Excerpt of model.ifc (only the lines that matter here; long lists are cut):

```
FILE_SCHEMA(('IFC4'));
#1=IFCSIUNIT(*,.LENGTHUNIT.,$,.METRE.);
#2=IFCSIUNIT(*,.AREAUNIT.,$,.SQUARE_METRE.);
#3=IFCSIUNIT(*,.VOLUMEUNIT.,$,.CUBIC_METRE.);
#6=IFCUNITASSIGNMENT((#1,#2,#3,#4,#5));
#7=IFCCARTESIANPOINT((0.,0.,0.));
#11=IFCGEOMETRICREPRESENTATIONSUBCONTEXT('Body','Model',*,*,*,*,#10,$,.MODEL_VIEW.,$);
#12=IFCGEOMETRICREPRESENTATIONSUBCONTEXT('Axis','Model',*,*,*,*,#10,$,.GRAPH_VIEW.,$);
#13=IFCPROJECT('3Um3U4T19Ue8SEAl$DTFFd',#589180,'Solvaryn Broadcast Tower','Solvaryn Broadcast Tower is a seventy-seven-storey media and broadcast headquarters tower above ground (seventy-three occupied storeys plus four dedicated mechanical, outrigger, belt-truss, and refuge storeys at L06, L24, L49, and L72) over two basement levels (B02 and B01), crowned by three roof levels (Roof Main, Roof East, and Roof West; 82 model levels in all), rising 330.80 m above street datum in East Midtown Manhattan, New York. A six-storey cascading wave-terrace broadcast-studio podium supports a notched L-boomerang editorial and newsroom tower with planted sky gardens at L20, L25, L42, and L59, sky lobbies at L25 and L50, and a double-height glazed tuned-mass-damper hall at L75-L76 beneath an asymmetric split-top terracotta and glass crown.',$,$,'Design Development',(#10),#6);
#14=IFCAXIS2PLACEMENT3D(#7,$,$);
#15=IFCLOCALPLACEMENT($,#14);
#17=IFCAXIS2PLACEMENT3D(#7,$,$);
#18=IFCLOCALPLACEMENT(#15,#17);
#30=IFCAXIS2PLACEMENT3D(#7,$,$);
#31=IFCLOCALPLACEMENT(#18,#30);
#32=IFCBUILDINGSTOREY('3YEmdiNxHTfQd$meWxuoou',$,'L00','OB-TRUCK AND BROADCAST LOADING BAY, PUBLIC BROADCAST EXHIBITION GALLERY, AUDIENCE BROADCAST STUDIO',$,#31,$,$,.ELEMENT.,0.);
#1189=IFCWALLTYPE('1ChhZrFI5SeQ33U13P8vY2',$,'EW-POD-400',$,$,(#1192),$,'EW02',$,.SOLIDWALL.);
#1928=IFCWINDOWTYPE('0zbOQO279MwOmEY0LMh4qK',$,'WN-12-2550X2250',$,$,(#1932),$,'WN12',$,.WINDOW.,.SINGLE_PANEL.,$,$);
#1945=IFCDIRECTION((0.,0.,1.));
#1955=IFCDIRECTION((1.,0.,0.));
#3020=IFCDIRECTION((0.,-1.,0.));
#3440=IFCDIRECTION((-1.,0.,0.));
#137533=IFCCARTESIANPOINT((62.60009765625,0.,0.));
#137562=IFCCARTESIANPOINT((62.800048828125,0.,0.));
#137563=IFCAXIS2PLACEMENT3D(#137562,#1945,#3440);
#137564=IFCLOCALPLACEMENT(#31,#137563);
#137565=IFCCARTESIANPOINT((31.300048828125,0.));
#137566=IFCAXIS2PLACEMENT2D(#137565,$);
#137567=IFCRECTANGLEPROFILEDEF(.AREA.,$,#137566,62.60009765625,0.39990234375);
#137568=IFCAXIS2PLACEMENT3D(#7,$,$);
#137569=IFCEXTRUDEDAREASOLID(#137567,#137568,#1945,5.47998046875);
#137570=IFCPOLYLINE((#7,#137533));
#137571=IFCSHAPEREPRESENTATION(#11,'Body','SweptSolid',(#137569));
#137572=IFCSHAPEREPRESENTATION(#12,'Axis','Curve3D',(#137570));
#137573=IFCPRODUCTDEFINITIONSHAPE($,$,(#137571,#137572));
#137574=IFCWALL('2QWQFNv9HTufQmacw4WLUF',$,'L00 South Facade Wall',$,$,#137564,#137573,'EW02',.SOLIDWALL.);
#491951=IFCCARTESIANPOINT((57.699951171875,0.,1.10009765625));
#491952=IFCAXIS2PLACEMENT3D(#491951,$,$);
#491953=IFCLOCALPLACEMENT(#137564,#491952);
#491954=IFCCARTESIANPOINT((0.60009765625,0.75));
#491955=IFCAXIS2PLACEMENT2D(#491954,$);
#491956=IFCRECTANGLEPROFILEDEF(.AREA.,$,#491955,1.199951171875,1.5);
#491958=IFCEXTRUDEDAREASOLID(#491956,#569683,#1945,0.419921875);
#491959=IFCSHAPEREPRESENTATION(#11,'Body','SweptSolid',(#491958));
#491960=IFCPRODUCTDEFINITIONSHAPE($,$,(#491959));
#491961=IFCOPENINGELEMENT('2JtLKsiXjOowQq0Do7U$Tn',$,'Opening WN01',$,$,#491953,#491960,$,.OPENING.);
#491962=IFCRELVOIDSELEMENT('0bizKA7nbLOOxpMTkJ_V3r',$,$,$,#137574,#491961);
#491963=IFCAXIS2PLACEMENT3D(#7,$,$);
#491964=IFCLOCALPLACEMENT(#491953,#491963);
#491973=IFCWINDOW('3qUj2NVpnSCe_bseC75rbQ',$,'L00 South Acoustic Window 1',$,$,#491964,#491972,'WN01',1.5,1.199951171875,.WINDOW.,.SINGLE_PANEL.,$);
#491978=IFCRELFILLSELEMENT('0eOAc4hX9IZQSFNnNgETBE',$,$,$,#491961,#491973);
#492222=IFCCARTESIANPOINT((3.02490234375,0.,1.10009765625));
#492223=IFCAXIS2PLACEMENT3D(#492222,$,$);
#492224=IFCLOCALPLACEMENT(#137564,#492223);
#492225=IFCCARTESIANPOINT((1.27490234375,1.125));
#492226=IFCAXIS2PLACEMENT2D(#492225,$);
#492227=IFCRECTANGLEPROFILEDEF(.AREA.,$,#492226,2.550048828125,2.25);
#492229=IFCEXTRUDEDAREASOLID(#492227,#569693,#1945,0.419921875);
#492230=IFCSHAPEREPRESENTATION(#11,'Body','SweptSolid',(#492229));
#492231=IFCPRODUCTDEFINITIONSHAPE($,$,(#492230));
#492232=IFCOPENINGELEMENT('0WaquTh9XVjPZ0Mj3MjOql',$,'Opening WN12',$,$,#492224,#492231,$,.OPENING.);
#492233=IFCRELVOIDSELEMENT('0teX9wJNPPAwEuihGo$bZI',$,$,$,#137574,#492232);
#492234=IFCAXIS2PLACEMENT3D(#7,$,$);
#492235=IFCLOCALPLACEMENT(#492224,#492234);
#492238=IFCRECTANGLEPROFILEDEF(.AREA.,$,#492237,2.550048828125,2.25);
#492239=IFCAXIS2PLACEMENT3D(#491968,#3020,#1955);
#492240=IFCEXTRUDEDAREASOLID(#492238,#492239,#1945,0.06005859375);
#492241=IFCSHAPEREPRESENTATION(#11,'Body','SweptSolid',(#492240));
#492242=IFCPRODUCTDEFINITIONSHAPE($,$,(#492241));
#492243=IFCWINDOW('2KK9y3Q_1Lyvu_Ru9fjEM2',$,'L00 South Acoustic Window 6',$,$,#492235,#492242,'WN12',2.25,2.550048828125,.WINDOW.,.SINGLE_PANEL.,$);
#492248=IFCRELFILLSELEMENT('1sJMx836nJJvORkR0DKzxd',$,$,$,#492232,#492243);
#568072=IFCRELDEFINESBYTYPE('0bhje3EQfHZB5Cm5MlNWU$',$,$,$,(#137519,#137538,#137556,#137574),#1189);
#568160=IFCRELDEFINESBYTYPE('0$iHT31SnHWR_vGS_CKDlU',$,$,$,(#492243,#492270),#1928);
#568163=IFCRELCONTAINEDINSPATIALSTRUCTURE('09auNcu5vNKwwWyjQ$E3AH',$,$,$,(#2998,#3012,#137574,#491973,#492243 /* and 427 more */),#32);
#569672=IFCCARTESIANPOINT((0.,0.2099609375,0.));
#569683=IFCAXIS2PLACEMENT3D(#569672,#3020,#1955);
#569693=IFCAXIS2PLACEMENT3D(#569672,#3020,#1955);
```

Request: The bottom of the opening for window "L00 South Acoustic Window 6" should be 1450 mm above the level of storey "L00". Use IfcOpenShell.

```python
import numpy as np
import ifcopenshell
import ifcopenshell.api.geometry
import ifcopenshell.geom
import ifcopenshell.util.element
import ifcopenshell.util.placement
import ifcopenshell.util.shape
import ifcopenshell.util.unit

model = ifcopenshell.open("model.ifc")
unit_scale = ifcopenshell.util.unit.calculate_unit_scale(model)

window = model.by_guid("2KK9y3Q_1Lyvu_Ru9fjEM2")
opening = window.FillsVoids[0].RelatingOpeningElement
storey = ifcopenshell.util.element.get_container(window, ifc_class="IfcBuildingStorey")
level = ifcopenshell.util.placement.get_local_placement(storey.ObjectPlacement)[2, 3]

# The opening's origin need not be at the sill, so measure its lowest point.
shape = ifcopenshell.geom.create_shape(ifcopenshell.geom.settings(), opening)
bottom = ifcopenshell.util.shape.get_shape_bottom_elevation(shape, shape.geometry) / unit_scale
dz = level + 1.45 / unit_scale - bottom

shift = np.array([0.0, 0.0, dz])
# The window is placed relative to its opening, so it follows when the opening moves.
matrix = ifcopenshell.util.placement.get_local_placement(opening.ObjectPlacement)
matrix[:3, 3] += shift
ifcopenshell.api.geometry.edit_object_placement(
    model, product=opening, matrix=matrix, is_si=False, should_transform_children=True
)

print(f"moved by {dz * unit_scale:+.3f} m")

model.write("model_rev.ifc")
```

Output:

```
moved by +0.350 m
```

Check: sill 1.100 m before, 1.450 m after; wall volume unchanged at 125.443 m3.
